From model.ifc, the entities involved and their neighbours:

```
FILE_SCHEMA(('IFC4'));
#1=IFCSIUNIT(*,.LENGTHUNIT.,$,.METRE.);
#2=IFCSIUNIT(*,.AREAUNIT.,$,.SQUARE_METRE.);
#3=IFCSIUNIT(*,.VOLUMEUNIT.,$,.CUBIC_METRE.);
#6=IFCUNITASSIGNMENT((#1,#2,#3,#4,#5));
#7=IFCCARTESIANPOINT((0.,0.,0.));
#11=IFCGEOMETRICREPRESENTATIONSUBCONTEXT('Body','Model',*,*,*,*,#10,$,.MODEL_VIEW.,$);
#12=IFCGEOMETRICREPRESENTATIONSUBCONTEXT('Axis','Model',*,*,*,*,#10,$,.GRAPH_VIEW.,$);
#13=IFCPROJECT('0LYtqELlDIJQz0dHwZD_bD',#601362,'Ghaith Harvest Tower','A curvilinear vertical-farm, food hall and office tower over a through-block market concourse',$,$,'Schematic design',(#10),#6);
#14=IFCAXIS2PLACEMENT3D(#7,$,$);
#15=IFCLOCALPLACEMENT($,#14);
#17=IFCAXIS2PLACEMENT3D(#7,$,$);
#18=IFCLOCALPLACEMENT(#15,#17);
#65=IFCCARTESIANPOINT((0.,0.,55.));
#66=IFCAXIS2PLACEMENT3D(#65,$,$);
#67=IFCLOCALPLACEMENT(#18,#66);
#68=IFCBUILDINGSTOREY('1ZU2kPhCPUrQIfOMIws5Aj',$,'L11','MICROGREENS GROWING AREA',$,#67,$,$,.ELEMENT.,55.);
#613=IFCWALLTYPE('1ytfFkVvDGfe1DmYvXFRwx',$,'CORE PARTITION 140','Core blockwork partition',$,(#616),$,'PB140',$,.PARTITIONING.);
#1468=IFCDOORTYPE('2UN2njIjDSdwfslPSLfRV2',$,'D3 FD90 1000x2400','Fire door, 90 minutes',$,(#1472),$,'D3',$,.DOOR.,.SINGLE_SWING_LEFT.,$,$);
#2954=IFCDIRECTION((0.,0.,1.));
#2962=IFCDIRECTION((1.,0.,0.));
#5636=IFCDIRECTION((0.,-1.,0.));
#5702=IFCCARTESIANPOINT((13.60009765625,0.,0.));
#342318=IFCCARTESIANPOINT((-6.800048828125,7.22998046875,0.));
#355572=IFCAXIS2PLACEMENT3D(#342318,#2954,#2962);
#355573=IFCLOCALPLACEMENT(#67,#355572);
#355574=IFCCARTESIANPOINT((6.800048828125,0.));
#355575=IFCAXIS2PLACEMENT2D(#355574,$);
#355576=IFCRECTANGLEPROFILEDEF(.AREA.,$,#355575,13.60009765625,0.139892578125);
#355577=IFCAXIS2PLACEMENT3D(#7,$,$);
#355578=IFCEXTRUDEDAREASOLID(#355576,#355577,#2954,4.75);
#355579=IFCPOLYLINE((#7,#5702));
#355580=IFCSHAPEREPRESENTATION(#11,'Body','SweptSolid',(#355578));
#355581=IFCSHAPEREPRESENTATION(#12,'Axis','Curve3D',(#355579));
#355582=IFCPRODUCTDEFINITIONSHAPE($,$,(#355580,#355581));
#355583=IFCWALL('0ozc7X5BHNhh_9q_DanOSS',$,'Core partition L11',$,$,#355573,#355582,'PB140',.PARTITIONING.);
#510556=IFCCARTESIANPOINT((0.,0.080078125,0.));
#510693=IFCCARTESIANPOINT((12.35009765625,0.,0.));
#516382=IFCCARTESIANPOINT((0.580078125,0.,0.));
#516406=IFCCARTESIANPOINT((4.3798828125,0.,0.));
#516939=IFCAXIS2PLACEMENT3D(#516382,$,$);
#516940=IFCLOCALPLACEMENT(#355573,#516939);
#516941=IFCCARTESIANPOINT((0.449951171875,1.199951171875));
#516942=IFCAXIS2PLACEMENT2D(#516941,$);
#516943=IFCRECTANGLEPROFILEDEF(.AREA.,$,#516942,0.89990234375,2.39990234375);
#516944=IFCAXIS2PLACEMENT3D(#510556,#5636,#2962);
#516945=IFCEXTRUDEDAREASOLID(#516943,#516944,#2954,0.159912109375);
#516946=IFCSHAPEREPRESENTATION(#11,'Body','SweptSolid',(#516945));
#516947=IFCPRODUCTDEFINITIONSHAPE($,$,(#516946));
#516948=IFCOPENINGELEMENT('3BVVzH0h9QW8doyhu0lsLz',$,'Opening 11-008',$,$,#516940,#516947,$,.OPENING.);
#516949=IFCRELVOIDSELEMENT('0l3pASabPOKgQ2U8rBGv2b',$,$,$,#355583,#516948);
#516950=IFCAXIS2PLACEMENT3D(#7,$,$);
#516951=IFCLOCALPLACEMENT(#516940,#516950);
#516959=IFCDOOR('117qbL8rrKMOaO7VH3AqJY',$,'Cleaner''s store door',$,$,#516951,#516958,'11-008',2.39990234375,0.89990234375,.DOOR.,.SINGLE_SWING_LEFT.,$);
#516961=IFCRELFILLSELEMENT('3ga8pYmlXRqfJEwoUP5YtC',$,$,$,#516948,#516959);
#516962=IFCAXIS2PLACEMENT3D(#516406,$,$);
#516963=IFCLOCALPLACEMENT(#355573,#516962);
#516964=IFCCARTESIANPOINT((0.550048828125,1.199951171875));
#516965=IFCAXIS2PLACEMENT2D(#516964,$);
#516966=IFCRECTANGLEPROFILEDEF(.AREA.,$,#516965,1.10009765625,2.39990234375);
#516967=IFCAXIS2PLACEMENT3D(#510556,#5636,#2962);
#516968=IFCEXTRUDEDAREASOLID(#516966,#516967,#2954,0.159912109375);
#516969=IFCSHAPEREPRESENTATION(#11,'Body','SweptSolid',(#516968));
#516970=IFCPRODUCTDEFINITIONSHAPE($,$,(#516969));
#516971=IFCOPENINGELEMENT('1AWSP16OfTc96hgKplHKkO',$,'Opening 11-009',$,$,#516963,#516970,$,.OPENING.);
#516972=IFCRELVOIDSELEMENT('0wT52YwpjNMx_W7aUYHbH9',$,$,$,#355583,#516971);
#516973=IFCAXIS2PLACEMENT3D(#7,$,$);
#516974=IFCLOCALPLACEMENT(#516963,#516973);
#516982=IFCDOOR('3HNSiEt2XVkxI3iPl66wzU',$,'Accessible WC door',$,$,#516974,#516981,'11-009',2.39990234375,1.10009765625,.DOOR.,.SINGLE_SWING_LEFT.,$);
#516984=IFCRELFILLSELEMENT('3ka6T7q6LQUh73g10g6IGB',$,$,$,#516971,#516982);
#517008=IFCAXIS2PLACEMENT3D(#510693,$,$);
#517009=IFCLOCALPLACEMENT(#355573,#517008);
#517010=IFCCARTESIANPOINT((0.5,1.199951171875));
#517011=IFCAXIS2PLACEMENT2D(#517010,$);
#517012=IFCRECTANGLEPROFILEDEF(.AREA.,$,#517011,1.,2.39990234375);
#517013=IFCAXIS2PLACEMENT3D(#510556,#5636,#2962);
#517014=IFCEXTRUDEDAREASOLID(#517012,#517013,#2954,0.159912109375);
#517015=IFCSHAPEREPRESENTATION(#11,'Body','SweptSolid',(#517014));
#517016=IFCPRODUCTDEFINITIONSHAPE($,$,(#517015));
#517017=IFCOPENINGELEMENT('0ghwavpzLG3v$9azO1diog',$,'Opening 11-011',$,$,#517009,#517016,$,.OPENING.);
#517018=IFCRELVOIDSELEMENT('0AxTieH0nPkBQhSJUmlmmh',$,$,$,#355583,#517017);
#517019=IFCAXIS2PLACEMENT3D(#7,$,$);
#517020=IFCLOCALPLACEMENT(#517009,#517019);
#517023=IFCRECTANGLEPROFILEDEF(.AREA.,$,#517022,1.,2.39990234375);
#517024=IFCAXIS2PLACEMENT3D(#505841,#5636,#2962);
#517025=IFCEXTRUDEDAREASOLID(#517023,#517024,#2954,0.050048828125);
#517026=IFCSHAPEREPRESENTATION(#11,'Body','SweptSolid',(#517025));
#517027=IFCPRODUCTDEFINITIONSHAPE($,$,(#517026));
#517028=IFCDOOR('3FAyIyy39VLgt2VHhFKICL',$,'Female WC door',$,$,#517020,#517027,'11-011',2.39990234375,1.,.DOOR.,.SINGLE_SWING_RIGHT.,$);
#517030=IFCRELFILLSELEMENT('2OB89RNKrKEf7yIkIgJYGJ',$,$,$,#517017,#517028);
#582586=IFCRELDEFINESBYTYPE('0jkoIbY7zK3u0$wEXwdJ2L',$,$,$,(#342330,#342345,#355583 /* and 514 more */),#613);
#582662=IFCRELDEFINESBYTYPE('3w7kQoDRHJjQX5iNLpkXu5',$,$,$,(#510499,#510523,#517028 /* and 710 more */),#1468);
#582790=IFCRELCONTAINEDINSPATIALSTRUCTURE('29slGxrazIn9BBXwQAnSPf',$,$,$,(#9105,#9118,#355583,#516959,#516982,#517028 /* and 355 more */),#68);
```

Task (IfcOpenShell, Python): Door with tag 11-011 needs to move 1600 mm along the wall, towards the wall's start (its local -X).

```python
import ifcopenshell
import ifcopenshell.api.geometry
import ifcopenshell.util.placement
import ifcopenshell.util.unit

model = ifcopenshell.open("model.ifc")
unit_scale = ifcopenshell.util.unit.calculate_unit_scale(model)

door = model.by_guid("3FAyIyy39VLgt2VHhFKICL")
opening = door.FillsVoids[0].RelatingOpeningElement
wall = opening.VoidsElements[0].RelatingBuildingElement

wall_matrix = ifcopenshell.util.placement.get_local_placement(wall.ObjectPlacement)
shift = wall_matrix[:3, 0] * -1.6 / unit_scale
before = ifcopenshell.util.placement.get_local_placement(door.ObjectPlacement)[:3, 3].copy()

# The door is placed relative to its opening, so it follows when the opening moves.
matrix = ifcopenshell.util.placement.get_local_placement(opening.ObjectPlacement)
matrix[:3, 3] += shift
ifcopenshell.api.geometry.edit_object_placement(
    model, product=opening, matrix=matrix, is_si=False, should_transform_children=True
)

after = ifcopenshell.util.placement.get_local_placement(door.ObjectPlacement)[:3, 3]
print("door moved by", (after - before).round(3) + 0.0)

model.write("model_edited.ifc")
```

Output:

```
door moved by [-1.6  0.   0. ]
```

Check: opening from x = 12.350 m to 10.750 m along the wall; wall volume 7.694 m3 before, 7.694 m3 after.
